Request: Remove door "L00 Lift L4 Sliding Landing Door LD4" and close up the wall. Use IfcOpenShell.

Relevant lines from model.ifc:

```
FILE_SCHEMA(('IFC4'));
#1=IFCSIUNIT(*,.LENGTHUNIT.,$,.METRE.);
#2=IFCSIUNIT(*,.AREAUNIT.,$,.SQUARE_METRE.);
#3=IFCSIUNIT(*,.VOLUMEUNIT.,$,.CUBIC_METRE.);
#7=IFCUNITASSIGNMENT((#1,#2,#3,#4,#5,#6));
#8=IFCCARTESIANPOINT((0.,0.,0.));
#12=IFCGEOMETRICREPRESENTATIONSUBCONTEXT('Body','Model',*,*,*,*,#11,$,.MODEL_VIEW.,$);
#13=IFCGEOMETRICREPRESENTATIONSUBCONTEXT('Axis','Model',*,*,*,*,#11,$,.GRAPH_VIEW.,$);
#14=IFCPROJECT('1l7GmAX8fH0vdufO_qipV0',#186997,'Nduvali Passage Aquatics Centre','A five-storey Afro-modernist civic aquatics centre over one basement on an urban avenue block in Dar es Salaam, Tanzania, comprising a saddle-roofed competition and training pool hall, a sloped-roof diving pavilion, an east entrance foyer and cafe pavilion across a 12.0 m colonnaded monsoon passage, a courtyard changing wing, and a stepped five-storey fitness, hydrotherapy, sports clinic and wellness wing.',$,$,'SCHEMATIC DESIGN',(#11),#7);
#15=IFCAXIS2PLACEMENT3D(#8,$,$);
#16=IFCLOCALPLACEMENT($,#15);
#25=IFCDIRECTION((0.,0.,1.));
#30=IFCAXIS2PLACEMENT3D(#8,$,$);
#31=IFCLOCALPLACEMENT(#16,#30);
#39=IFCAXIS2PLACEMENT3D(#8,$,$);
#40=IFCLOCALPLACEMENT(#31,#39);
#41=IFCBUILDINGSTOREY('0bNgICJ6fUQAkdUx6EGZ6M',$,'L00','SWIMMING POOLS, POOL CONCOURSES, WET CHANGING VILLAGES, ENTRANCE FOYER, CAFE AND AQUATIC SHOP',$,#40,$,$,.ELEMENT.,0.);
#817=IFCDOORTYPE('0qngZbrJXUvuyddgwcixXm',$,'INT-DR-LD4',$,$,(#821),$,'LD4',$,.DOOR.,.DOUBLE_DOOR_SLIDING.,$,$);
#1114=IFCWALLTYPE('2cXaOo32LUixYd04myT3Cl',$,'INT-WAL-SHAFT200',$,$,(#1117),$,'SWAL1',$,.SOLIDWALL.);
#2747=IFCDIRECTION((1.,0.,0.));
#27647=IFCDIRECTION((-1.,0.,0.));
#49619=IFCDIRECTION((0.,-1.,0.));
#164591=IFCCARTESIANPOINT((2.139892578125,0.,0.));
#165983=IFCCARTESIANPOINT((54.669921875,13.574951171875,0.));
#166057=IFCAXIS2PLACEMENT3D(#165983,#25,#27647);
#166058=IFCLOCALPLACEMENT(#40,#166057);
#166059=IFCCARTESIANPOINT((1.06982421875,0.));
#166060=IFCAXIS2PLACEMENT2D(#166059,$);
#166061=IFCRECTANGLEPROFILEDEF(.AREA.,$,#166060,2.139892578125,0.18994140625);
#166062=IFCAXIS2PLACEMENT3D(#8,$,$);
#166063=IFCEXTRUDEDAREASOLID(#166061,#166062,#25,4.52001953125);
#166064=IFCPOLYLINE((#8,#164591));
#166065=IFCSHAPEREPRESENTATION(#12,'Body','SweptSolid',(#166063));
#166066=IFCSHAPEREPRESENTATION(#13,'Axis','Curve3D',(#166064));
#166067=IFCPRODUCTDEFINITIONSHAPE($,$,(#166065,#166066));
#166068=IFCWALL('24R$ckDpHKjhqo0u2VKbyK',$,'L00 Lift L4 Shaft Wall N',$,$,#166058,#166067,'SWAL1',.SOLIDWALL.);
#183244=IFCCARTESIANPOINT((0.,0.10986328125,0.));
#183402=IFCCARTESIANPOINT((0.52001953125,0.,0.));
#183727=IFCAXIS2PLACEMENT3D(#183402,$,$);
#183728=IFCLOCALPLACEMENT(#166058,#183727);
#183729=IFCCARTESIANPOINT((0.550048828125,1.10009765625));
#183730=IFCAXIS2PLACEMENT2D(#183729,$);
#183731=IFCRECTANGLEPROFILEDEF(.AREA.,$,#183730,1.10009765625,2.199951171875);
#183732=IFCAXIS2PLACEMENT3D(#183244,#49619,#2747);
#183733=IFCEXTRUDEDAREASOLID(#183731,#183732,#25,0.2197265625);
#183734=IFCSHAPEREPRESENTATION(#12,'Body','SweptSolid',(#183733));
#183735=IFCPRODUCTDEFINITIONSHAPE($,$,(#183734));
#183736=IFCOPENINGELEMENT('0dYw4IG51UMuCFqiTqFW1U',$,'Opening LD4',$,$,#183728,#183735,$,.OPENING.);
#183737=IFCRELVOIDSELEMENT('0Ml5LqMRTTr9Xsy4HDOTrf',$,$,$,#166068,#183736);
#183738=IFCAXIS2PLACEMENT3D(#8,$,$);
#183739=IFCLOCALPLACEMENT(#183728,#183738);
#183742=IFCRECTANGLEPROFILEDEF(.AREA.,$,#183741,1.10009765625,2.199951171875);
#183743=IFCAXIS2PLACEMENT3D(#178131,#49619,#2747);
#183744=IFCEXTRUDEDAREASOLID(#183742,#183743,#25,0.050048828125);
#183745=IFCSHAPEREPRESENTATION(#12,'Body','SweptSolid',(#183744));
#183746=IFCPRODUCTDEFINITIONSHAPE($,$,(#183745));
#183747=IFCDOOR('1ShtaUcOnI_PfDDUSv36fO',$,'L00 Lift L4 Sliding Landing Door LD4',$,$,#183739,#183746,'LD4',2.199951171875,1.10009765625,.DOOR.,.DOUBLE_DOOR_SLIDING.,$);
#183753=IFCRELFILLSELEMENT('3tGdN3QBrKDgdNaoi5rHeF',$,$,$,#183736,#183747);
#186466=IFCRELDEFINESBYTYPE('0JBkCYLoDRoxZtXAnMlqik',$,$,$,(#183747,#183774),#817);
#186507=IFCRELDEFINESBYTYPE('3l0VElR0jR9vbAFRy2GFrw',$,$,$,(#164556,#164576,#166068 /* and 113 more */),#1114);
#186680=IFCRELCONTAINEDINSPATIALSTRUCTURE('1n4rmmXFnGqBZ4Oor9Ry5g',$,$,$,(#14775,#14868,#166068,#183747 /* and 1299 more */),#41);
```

```python
import ifcopenshell
import ifcopenshell.api.feature
import ifcopenshell.api.root
import ifcopenshell.geom
import ifcopenshell.util.shape

model = ifcopenshell.open("model.ifc")
settings = ifcopenshell.geom.settings()


def volume(element):
    """Net volume in cubic metres, openings subtracted."""
    shape = ifcopenshell.geom.create_shape(settings, element)
    return ifcopenshell.util.shape.get_volume(shape.geometry)


door = model.by_guid("1ShtaUcOnI_PfDDUSv36fO")
opening = door.FillsVoids[0].RelatingOpeningElement
wall = opening.VoidsElements[0].RelatingBuildingElement
before = volume(wall)

ifcopenshell.api.root.remove_product(model, product=door)
ifcopenshell.api.feature.remove_feature(model, feature=opening)

after = volume(wall)

print(f"wall volume {before:.3f} -> {after:.3f} m3")

model.write("model-out.ifc")
```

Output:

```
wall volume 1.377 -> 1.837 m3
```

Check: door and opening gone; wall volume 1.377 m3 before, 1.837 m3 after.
